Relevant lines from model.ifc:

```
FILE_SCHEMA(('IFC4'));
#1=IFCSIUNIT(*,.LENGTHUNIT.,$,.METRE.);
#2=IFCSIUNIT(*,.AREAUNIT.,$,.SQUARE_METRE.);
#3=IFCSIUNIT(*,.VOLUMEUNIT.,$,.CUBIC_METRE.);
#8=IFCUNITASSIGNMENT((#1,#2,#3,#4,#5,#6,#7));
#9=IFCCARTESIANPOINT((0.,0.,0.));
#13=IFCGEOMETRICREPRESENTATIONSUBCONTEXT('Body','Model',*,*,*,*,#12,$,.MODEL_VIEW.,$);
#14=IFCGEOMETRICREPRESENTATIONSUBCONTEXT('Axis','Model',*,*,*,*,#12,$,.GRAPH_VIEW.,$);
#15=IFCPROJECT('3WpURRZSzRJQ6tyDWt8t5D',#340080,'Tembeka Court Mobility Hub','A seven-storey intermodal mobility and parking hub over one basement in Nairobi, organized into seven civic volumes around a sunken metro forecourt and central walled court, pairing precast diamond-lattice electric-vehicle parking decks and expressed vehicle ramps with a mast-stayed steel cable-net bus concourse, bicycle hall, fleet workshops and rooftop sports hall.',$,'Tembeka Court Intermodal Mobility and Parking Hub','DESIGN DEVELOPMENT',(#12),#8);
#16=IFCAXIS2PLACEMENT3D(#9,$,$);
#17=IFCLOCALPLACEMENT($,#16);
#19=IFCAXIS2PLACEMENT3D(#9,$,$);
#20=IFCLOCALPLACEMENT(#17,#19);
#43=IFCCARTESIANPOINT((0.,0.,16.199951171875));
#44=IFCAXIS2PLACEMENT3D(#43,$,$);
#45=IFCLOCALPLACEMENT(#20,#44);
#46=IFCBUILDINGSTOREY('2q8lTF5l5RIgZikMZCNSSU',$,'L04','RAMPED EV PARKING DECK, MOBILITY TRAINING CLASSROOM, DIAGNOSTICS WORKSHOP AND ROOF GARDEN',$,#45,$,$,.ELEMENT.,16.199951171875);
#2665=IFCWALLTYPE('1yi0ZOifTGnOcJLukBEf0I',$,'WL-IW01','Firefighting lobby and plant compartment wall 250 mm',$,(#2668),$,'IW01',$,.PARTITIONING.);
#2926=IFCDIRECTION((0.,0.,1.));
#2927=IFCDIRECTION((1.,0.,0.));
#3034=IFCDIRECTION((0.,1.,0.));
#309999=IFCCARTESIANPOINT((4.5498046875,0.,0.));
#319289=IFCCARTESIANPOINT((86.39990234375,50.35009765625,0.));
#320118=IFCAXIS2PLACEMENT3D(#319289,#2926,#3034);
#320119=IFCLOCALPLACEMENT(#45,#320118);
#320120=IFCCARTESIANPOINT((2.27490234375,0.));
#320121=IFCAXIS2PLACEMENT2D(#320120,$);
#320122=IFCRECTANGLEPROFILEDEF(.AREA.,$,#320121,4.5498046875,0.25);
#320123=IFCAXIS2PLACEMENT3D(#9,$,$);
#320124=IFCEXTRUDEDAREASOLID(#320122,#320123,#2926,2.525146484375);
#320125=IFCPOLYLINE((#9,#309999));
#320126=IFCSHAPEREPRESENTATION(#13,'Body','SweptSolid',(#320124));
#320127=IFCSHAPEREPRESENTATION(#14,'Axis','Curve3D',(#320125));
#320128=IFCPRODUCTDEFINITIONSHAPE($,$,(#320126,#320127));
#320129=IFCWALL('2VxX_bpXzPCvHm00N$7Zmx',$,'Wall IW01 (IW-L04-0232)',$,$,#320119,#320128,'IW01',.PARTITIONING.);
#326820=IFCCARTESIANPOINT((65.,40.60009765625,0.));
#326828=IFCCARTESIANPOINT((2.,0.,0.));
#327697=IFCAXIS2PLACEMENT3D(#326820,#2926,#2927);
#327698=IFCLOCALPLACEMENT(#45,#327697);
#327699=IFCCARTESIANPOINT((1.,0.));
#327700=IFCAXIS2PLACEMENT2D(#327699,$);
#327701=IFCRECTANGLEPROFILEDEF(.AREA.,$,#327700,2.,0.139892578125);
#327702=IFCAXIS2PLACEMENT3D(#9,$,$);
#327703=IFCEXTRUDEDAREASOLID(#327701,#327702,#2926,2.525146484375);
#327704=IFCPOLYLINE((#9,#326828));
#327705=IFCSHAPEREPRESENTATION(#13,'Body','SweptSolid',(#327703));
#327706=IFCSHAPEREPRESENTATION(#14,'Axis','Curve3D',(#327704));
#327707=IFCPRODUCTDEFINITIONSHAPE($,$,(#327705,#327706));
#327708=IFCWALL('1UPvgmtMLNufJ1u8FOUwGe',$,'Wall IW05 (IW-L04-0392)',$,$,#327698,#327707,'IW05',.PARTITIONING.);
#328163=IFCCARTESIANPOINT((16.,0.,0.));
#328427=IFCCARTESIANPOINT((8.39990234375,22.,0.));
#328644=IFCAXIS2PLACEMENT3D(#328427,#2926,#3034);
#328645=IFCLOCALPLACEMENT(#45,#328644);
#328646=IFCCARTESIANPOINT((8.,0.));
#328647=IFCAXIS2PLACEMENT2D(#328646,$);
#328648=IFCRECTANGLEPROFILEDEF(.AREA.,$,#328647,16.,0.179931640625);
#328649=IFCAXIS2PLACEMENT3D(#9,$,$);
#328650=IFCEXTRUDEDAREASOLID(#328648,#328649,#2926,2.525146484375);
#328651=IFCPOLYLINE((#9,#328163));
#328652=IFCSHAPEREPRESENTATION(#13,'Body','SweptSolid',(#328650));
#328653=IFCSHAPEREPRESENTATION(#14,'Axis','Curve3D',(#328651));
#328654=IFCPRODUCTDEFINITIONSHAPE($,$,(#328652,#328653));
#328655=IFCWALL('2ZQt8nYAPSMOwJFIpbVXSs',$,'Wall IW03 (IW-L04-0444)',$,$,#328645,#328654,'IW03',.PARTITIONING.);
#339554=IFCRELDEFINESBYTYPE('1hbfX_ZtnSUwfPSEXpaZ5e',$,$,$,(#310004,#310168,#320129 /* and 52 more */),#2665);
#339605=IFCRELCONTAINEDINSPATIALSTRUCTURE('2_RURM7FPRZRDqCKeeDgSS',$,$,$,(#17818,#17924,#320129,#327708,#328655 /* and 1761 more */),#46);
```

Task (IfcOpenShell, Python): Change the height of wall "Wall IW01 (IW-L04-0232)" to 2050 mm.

```python
import ifcopenshell
import ifcopenshell.geom
import ifcopenshell.util.representation
import ifcopenshell.util.shape

model = ifcopenshell.open("model.ifc")
settings = ifcopenshell.geom.settings()


def volume(element):
    """Net volume in cubic metres, openings subtracted."""
    shape = ifcopenshell.geom.create_shape(settings, element)
    return ifcopenshell.util.shape.get_volume(shape.geometry)


wall = model.by_guid("2VxX_bpXzPCvHm00N$7Zmx")
before = volume(wall)

body = ifcopenshell.util.representation.get_representation(wall, "Model", "Body")
solid = body.Items[0]
old_height = solid.Depth
solid.Depth = 2.05
after = volume(wall)

print(f"height {old_height:g} -> {solid.Depth:g}, volume {before:.3f} -> {after:.3f} m3")

model.write("model_edited.ifc")
```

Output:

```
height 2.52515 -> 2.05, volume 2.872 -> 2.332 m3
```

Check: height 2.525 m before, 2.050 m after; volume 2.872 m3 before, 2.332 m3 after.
